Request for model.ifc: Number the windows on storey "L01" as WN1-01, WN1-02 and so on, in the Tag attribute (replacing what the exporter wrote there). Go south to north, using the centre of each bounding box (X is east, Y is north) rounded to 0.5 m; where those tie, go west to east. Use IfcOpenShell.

First a look at what the model holds.

```python
import ifcopenshell
import ifcopenshell.util.element
import ifcopenshell.util.placement

model = ifcopenshell.open("model.ifc")
print(model.schema)
storey = next(s for s in model.by_type("IfcBuildingStorey") if s.Name == "L01")
windows = [e for e in ifcopenshell.util.element.get_decomposition(storey) if e.is_a("IfcWindow")]
for e in sorted(windows, key=lambda e: e.id()):
    origin = ifcopenshell.util.placement.get_local_placement(e.ObjectPlacement)[:3, 3]
    print(e.id(), e.Tag, e.Name, origin.round(2) + 0.0, sep=" | ")
```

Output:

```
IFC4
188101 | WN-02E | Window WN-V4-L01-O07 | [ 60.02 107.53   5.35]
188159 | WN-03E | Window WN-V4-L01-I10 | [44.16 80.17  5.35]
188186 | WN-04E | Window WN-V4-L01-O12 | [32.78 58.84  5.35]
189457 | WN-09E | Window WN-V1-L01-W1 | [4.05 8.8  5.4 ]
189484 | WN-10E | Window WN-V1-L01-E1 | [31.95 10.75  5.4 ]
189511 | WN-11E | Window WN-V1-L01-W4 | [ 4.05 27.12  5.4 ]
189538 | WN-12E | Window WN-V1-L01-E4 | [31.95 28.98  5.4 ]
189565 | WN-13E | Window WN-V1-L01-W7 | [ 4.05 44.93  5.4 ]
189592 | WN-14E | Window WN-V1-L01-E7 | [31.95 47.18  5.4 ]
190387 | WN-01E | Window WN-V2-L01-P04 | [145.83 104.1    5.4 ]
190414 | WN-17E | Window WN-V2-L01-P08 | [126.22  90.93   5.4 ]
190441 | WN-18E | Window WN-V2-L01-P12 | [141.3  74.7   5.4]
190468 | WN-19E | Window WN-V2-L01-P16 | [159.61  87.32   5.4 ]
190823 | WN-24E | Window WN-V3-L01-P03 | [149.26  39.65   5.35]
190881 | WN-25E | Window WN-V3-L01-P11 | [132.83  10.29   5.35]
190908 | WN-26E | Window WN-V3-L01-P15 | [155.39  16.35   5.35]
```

```python
import ifcopenshell
import ifcopenshell.geom
import ifcopenshell.util.element
import ifcopenshell.util.shape

model = ifcopenshell.open("model.ifc")
settings = ifcopenshell.geom.settings()
settings.set("use-world-coords", True)


def centre(element):
    shape = ifcopenshell.geom.create_shape(settings, element)
    return ifcopenshell.util.shape.get_bbox_centroid(shape.geometry)


storey = next(s for s in model.by_type("IfcBuildingStorey") if s.Name == "L01")
windows = [e for e in ifcopenshell.util.element.get_decomposition(storey) if e.is_a("IfcWindow")]

# Insertion points can sit at a corner or the storey origin, so sort by the geometry (in metres).
centres = {e: centre(e) for e in windows}
windows.sort(key=lambda e: (round(centres[e][1] / 0.5), centres[e][0]))

for i, e in enumerate(windows, start=1):
    number = f"WN1-{i:02d}"
    e.Tag = number
    print(e.id(), number)

model.write("model_v2.ifc")
```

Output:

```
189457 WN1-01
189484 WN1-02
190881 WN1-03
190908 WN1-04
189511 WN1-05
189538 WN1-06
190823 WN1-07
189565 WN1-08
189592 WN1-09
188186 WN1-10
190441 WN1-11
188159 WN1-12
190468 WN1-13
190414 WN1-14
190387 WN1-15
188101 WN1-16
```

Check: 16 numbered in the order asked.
